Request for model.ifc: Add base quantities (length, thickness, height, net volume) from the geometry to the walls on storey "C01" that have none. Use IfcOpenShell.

First a look at what the model holds.

```python
import ifcopenshell
import ifcopenshell.util.element
import ifcopenshell.util.unit

model = ifcopenshell.open("model.ifc")
print(model.schema)
for unit_type in ("LENGTHUNIT", "AREAUNIT", "VOLUMEUNIT"):
    print(unit_type, ifcopenshell.util.unit.calculate_unit_scale(model, unit_type))
storey = next(s for s in model.by_type("IfcBuildingStorey") if s.Name == "C01")
walls = [e for e in ifcopenshell.util.element.get_decomposition(storey) if e.is_a("IfcWall")]
for e in sorted(walls, key=lambda e: e.id()):
    print(e.id(), e.is_a(), e.Name, list(ifcopenshell.util.element.get_psets(e, qtos_only=True)), sep=" | ")
```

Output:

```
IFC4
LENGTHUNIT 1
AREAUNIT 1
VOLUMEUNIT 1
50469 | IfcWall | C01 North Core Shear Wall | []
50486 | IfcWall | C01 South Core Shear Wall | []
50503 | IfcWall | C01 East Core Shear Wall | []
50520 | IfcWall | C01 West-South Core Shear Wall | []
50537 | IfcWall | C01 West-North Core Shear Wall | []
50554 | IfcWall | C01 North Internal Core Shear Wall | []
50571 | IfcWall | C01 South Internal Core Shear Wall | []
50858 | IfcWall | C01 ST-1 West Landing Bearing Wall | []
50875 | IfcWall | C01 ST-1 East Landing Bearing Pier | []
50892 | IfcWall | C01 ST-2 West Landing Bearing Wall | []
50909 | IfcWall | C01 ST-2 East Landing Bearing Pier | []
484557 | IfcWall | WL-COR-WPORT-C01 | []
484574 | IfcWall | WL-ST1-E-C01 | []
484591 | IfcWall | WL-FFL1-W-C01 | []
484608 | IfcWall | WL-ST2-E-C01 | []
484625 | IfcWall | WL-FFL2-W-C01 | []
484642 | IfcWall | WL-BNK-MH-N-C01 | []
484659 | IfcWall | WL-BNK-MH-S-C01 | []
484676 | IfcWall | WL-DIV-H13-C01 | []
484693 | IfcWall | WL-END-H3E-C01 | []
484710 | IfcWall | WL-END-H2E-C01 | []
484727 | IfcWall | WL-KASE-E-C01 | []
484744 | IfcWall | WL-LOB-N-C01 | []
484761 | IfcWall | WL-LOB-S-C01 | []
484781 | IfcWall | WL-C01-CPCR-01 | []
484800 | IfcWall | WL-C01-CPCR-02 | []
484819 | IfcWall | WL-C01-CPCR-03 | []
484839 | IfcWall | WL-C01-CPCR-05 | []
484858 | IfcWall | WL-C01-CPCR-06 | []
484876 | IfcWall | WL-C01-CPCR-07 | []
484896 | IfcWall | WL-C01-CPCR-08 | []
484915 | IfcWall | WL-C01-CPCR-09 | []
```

```python
import ifcopenshell
import ifcopenshell.api.pset
import ifcopenshell.geom
import ifcopenshell.util.element
import ifcopenshell.util.shape
import ifcopenshell.util.unit

model = ifcopenshell.open("model.ifc")
unit_scale = ifcopenshell.util.unit.calculate_unit_scale(model)
volume_scale = ifcopenshell.util.unit.calculate_unit_scale(model, "VOLUMEUNIT")
settings = ifcopenshell.geom.settings()

storey = next(s for s in model.by_type("IfcBuildingStorey") if s.Name == "C01")
walls = [e for e in ifcopenshell.util.element.get_decomposition(storey) if e.is_a("IfcWall")]

for e in sorted(walls, key=lambda e: e.id()):
    if ifcopenshell.util.element.get_psets(e, qtos_only=True, should_inherit=False):
        continue
    # Geometry comes back in metres, in the element's own axes.
    shape = ifcopenshell.geom.create_shape(settings, e)
    values = {
        "Length": ifcopenshell.util.shape.get_x(shape.geometry) / unit_scale,
        "Width": ifcopenshell.util.shape.get_y(shape.geometry) / unit_scale,
        "Height": ifcopenshell.util.shape.get_z(shape.geometry) / unit_scale,
        "NetVolume": ifcopenshell.util.shape.get_volume(shape.geometry) / volume_scale,
    }
    qto = ifcopenshell.api.pset.add_qto(model, product=e, name="Qto_WallBaseQuantities")
    ifcopenshell.api.pset.edit_qto(model, qto=qto, properties=values)
    print(e.id(), {k: round(v, 3) for k, v in values.items()})

model.write("model_updated.ifc")
```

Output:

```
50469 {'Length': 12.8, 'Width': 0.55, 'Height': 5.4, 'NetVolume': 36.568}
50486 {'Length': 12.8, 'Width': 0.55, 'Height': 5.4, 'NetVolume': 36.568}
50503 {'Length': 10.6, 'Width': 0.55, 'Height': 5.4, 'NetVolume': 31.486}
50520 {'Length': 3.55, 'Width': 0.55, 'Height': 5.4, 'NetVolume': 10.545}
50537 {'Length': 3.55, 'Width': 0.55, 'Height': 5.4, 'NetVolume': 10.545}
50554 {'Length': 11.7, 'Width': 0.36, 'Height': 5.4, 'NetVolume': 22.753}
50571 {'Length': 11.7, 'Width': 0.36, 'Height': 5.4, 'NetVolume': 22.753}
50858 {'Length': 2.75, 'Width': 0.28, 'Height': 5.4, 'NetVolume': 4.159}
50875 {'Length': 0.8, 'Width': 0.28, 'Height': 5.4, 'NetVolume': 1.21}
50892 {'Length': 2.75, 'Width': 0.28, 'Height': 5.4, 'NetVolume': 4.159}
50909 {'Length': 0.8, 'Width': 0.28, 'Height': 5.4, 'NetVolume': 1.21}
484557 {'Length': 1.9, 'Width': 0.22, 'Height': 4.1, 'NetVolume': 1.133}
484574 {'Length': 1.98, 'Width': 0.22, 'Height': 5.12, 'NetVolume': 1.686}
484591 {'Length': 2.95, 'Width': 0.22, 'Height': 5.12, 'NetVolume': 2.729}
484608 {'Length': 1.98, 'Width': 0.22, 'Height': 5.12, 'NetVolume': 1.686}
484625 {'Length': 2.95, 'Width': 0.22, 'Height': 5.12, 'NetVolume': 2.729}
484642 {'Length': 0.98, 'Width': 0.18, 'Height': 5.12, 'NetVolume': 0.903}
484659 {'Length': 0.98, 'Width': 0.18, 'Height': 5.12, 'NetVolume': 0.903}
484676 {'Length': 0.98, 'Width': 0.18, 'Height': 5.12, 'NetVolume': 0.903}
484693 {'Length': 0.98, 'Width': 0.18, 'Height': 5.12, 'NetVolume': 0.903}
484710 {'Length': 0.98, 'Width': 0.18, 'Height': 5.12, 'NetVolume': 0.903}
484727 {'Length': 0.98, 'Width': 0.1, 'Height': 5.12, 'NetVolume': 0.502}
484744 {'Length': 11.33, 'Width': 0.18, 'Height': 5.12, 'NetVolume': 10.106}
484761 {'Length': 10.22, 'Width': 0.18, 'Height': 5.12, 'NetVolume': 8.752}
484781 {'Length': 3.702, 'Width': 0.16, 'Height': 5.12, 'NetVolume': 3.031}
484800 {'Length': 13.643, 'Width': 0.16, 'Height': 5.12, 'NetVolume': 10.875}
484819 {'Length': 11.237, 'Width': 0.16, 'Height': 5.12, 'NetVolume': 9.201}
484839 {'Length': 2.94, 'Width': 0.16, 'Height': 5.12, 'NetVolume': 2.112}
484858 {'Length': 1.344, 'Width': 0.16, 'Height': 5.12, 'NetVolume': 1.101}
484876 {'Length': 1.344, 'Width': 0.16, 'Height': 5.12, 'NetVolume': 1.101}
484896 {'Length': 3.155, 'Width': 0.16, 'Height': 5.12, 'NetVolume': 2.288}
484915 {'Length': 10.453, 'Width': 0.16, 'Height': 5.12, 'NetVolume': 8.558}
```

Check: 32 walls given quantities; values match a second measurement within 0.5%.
